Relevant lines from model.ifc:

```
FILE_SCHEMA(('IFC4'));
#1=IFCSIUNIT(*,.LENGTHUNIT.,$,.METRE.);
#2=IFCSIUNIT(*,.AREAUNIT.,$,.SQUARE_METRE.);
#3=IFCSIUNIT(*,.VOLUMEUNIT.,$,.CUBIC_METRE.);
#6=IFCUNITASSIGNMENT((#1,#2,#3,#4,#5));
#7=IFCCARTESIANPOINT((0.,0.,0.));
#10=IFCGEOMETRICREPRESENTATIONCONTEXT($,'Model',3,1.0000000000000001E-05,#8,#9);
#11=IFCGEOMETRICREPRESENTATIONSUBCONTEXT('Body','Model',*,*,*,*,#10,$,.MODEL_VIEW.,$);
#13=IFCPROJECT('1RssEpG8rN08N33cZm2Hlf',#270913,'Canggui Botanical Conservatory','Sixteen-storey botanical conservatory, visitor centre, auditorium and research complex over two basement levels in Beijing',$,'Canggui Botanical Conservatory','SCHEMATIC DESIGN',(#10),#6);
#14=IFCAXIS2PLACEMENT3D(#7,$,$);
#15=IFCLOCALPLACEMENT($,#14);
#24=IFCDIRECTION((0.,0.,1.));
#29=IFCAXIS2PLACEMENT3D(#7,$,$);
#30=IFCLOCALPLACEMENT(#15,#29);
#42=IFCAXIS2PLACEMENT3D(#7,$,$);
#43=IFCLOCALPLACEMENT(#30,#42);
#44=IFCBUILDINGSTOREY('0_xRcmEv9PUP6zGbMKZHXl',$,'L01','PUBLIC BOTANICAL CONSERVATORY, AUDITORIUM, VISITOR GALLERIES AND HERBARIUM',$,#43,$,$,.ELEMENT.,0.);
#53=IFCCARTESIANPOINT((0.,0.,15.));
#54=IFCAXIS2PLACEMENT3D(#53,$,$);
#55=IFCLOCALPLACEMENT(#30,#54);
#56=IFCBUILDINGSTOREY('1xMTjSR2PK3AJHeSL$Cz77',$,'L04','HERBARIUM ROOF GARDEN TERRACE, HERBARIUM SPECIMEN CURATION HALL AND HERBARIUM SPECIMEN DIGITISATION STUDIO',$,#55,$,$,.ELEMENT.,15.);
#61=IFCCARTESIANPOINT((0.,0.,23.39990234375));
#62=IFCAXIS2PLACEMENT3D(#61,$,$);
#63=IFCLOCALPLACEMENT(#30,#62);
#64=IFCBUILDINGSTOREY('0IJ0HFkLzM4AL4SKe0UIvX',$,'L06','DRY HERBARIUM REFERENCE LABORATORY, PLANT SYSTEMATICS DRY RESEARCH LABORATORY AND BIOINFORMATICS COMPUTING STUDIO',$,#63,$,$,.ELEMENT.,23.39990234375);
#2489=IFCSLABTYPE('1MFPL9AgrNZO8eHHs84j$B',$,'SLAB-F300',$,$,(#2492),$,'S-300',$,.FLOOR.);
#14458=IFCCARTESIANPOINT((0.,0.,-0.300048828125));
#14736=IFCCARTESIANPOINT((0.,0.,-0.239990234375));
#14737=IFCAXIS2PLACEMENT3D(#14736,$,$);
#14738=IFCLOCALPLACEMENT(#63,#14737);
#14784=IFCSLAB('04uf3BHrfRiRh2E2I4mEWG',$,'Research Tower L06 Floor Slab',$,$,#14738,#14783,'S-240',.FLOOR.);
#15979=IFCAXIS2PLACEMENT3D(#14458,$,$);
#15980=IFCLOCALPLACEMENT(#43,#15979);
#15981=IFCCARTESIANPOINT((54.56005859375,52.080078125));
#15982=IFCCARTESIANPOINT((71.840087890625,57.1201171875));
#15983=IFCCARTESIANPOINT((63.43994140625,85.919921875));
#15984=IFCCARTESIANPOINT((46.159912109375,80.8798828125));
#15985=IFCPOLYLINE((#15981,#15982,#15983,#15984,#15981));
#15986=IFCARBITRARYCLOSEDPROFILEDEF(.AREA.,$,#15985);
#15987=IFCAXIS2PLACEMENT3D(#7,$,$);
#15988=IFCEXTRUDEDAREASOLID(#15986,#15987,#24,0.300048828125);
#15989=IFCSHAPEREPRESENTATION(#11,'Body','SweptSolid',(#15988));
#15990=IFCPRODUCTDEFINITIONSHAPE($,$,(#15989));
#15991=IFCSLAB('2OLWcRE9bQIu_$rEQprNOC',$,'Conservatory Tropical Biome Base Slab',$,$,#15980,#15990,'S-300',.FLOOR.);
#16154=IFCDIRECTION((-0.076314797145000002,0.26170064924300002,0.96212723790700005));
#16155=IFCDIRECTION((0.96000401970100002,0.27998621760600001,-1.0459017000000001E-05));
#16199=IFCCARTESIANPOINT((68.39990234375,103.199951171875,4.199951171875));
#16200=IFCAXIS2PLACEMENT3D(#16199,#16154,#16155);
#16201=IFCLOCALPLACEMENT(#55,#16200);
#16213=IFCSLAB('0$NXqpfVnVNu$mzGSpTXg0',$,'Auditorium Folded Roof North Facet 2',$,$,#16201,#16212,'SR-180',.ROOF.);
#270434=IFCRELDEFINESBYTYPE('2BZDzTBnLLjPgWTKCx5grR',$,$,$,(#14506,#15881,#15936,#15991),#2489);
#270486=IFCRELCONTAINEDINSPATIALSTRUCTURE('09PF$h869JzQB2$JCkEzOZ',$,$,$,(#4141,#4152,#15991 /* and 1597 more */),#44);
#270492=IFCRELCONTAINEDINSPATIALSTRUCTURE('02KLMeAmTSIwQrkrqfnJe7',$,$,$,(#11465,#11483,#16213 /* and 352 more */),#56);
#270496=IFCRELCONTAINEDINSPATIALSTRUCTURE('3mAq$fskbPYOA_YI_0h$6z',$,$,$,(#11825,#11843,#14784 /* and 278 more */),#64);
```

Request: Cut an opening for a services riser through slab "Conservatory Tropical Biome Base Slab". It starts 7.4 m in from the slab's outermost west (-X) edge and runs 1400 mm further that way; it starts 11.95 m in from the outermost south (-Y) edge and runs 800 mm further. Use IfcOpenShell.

```python
import numpy as np
import ifcopenshell
import ifcopenshell.api.feature
import ifcopenshell.api.geometry
import ifcopenshell.api.root
import ifcopenshell.geom
import ifcopenshell.util.placement
import ifcopenshell.util.representation
import ifcopenshell.util.shape
import ifcopenshell.util.unit

model = ifcopenshell.open("model.ifc")
unit_scale = ifcopenshell.util.unit.calculate_unit_scale(model)
settings = ifcopenshell.geom.settings()


def volume(element):
    """Net volume in cubic metres, openings subtracted."""
    shape = ifcopenshell.geom.create_shape(settings, element)
    return ifcopenshell.util.shape.get_volume(shape.geometry)


slab = model.by_guid("2OLWcRE9bQIu_$rEQprNOC")
before = volume(slab)

# Extent in the slab's own axes, in metres. The edges named are its -X and -Y sides.
slab_shape = ifcopenshell.geom.create_shape(settings, slab)
vertices = ifcopenshell.util.shape.get_vertices(slab_shape.geometry)
x_min, y_min, bottom = vertices.min(axis=0)
top = vertices[:, 2].max()

opening = ifcopenshell.api.root.create_entity(model, ifc_class="IfcOpeningElement", name="Services riser opening", predefined_type="OPENING")
context = ifcopenshell.util.representation.get_context(model, "Model", "Body", "MODEL_VIEW")
width, depth = 1.4, 0.8
outline = [(0.0, 0.0), (width, 0.0), (width, depth), (0.0, depth), (0.0, 0.0)]
# Overshoot both faces by 50 mm so the cut is clean.
shape = ifcopenshell.api.geometry.add_slab_representation(
    model, context=context, depth=top - bottom + 0.1, polyline=outline
)
ifcopenshell.api.geometry.assign_representation(model, product=opening, representation=shape)

matrix = ifcopenshell.util.placement.get_local_placement(slab.ObjectPlacement)
matrix[:, 3] = matrix @ np.append(np.array([x_min + 7.4, y_min + 11.95, bottom - 0.05]) / unit_scale, 1.0)
ifcopenshell.api.geometry.edit_object_placement(model, product=opening, matrix=matrix, is_si=False)
ifcopenshell.api.feature.add_feature(model, feature=opening, element=slab)

after = volume(slab)

print(f"slab volume {before:.3f} -> {after:.3f} m3")

model.write("model_edited.ifc")
```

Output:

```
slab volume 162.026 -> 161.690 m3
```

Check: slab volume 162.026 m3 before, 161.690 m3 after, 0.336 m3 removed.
